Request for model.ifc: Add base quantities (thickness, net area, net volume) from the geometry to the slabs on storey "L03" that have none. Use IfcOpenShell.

First a look at what the model holds.

```python
import ifcopenshell
import ifcopenshell.util.element
import ifcopenshell.util.unit

model = ifcopenshell.open("model.ifc")
print(model.schema)
for unit_type in ("LENGTHUNIT", "AREAUNIT", "VOLUMEUNIT"):
    print(unit_type, ifcopenshell.util.unit.calculate_unit_scale(model, unit_type))
storey = next(s for s in model.by_type("IfcBuildingStorey") if s.Name == "L03")
slabs = [e for e in ifcopenshell.util.element.get_decomposition(storey) if e.is_a("IfcSlab")]
for e in sorted(slabs, key=lambda e: e.id()):
    print(e.id(), e.is_a(), e.Name, list(ifcopenshell.util.element.get_psets(e, qtos_only=True)), sep=" | ")
```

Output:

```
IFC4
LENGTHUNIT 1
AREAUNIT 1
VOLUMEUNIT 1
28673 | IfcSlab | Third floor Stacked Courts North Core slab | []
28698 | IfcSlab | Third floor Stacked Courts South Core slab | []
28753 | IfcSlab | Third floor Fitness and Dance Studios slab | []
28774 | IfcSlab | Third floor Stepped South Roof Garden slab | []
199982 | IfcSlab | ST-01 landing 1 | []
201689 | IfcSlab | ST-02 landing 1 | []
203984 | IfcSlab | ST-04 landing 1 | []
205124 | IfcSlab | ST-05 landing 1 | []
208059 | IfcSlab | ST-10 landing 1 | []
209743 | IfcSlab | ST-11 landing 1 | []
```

```python
import ifcopenshell
import ifcopenshell.api.pset
import ifcopenshell.geom
import ifcopenshell.util.element
import ifcopenshell.util.shape
import ifcopenshell.util.unit

model = ifcopenshell.open("model.ifc")
unit_scale = ifcopenshell.util.unit.calculate_unit_scale(model)
area_scale = ifcopenshell.util.unit.calculate_unit_scale(model, "AREAUNIT")
volume_scale = ifcopenshell.util.unit.calculate_unit_scale(model, "VOLUMEUNIT")
settings = ifcopenshell.geom.settings()

storey = next(s for s in model.by_type("IfcBuildingStorey") if s.Name == "L03")
slabs = [e for e in ifcopenshell.util.element.get_decomposition(storey) if e.is_a("IfcSlab")]

for e in sorted(slabs, key=lambda e: e.id()):
    if ifcopenshell.util.element.get_psets(e, qtos_only=True, should_inherit=False):
        continue
    # Geometry comes back in metres, in the element's own axes.
    shape = ifcopenshell.geom.create_shape(settings, e)
    values = {
        "Width": ifcopenshell.util.shape.get_z(shape.geometry) / unit_scale,
        "NetArea": ifcopenshell.util.shape.get_footprint_area(shape.geometry) / area_scale,
        "NetVolume": ifcopenshell.util.shape.get_volume(shape.geometry) / volume_scale,
    }
    qto = ifcopenshell.api.pset.add_qto(model, product=e, name="Qto_SlabBaseQuantities")
    ifcopenshell.api.pset.edit_qto(model, qto=qto, properties=values)
    print(e.id(), {k: round(v, 3) for k, v in values.items()})

model.write("model_v2.ifc")
```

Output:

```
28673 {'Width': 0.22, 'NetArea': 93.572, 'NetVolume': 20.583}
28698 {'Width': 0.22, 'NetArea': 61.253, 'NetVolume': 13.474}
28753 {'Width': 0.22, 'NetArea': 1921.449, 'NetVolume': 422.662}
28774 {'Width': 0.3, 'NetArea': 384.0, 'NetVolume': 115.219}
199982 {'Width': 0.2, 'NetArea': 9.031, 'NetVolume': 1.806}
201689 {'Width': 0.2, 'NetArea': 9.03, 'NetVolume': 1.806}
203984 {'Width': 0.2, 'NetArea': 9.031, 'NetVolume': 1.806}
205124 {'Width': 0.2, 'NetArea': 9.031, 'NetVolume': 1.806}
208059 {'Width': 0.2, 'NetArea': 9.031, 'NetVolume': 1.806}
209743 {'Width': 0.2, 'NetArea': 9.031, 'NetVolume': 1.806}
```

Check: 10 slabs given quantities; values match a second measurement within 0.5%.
